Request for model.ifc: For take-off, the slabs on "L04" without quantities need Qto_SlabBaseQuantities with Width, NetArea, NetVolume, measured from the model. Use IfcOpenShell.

First a look at what the model holds.

```python
import ifcopenshell
import ifcopenshell.util.element
import ifcopenshell.util.unit

model = ifcopenshell.open("model.ifc")
print(model.schema)
for unit_type in ("LENGTHUNIT", "AREAUNIT", "VOLUMEUNIT"):
    print(unit_type, ifcopenshell.util.unit.calculate_unit_scale(model, unit_type))
storey = next(s for s in model.by_type("IfcBuildingStorey") if s.Name == "L04")
slabs = [e for e in ifcopenshell.util.element.get_decomposition(storey) if e.is_a("IfcSlab")]
for e in sorted(slabs, key=lambda e: e.id()):
    print(e.id(), e.is_a(), e.Name, list(ifcopenshell.util.element.get_psets(e, qtos_only=True)), sep=" | ")
```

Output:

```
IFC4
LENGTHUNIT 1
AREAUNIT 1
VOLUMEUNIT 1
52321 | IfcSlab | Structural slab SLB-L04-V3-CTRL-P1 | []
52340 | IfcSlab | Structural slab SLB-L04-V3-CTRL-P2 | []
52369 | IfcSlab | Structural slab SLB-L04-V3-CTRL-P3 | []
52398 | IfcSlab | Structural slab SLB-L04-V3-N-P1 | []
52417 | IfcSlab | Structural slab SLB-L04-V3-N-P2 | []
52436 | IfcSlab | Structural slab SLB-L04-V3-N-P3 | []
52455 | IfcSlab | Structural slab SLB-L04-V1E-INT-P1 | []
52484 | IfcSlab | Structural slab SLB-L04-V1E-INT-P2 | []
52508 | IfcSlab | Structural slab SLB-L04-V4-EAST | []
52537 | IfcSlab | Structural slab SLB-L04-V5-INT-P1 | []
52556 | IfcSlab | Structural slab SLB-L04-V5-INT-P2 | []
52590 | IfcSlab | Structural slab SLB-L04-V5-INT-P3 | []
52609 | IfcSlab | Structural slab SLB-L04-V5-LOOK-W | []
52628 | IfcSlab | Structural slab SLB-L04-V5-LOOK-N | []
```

```python
import ifcopenshell
import ifcopenshell.api.pset
import ifcopenshell.geom
import ifcopenshell.util.element
import ifcopenshell.util.shape
import ifcopenshell.util.unit

model = ifcopenshell.open("model.ifc")
unit_scale = ifcopenshell.util.unit.calculate_unit_scale(model)
area_scale = ifcopenshell.util.unit.calculate_unit_scale(model, "AREAUNIT")
volume_scale = ifcopenshell.util.unit.calculate_unit_scale(model, "VOLUMEUNIT")
settings = ifcopenshell.geom.settings()

storey = next(s for s in model.by_type("IfcBuildingStorey") if s.Name == "L04")
slabs = [e for e in ifcopenshell.util.element.get_decomposition(storey) if e.is_a("IfcSlab")]

for e in sorted(slabs, key=lambda e: e.id()):
    if ifcopenshell.util.element.get_psets(e, qtos_only=True, should_inherit=False):
        continue
    # Geometry comes back in metres, in the element's own axes.
    shape = ifcopenshell.geom.create_shape(settings, e)
    values = {
        "Width": ifcopenshell.util.shape.get_z(shape.geometry) / unit_scale,
        "NetArea": ifcopenshell.util.shape.get_footprint_area(shape.geometry) / area_scale,
        "NetVolume": ifcopenshell.util.shape.get_volume(shape.geometry) / volume_scale,
    }
    qto = ifcopenshell.api.pset.add_qto(model, product=e, name="Qto_SlabBaseQuantities")
    ifcopenshell.api.pset.edit_qto(model, qto=qto, properties=values)
    print(e.id(), {k: round(v, 3) for k, v in values.items()})

model.write("model_edited.ifc")
```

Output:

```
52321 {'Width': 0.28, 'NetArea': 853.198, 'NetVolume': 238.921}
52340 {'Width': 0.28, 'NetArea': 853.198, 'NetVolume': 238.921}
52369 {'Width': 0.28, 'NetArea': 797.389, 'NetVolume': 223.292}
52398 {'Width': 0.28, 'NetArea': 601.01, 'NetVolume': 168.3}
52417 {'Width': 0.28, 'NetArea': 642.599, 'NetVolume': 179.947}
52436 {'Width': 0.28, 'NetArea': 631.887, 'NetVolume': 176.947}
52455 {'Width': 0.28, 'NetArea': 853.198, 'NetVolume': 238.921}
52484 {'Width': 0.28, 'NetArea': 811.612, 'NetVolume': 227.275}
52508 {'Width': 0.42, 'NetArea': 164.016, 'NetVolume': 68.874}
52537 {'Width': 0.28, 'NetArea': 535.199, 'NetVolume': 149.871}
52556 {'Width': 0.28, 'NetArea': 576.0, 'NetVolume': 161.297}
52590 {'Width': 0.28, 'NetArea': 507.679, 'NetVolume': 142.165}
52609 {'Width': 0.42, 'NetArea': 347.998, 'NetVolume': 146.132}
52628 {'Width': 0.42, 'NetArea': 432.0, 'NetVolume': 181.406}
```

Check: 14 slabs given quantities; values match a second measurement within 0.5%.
